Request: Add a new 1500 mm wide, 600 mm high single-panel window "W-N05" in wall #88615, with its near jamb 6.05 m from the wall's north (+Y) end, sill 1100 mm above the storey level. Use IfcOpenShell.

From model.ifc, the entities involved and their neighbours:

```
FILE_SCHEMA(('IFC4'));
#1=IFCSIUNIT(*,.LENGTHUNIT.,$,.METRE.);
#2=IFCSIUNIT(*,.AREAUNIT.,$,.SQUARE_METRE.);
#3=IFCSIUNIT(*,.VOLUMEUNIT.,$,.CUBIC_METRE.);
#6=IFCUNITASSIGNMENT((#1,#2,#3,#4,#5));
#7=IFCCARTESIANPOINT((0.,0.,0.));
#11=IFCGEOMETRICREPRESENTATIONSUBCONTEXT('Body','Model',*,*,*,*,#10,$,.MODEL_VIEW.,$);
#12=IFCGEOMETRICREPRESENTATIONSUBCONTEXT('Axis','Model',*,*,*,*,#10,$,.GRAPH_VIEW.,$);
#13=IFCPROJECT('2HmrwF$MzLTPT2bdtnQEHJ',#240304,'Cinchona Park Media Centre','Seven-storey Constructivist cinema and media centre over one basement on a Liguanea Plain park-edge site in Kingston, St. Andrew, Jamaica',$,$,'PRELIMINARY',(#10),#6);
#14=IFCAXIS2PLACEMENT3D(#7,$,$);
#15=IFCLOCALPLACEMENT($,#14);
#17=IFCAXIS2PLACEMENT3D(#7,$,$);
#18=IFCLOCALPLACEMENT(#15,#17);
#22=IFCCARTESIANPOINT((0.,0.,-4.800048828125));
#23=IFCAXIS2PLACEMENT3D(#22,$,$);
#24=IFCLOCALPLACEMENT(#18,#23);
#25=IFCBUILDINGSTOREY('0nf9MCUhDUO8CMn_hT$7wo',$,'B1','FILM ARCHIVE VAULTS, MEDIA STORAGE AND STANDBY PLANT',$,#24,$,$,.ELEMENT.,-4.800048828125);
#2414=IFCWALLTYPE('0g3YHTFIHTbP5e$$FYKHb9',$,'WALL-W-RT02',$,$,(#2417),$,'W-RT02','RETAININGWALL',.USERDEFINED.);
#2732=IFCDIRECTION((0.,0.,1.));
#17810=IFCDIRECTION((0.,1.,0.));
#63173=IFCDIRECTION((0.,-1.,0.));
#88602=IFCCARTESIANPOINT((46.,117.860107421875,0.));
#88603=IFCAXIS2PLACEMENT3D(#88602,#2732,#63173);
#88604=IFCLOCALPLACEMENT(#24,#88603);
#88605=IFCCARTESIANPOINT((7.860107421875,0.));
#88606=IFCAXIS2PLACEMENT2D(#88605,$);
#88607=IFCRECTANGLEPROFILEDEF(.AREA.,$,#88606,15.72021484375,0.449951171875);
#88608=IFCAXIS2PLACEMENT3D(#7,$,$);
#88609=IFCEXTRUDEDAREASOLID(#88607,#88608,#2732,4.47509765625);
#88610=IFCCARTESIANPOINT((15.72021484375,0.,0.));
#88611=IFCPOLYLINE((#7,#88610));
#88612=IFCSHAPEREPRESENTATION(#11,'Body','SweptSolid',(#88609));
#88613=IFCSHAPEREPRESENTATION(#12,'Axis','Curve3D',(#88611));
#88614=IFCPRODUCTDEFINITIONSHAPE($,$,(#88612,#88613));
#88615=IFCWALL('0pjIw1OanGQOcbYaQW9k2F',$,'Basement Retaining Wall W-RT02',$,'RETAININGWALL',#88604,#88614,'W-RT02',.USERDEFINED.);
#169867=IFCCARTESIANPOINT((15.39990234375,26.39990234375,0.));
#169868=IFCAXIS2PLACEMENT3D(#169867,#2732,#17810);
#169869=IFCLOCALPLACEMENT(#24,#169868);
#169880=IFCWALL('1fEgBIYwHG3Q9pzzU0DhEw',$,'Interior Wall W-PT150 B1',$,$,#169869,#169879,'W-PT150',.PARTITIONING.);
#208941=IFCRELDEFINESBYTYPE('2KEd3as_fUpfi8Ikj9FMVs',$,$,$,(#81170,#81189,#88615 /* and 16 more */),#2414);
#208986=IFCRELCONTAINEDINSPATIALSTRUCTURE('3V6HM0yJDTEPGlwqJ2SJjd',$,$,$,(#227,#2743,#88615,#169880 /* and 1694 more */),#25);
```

```python
import numpy as np
import ifcopenshell
import ifcopenshell.api.feature
import ifcopenshell.api.geometry
import ifcopenshell.api.root
import ifcopenshell.api.spatial
import ifcopenshell.geom
import ifcopenshell.util.element
import ifcopenshell.util.placement
import ifcopenshell.util.representation
import ifcopenshell.util.shape
import ifcopenshell.util.unit

model = ifcopenshell.open("model.ifc")
unit_scale = ifcopenshell.util.unit.calculate_unit_scale(model)
settings = ifcopenshell.geom.settings()


def volume(element):
    """Net volume in cubic metres, openings subtracted."""
    shape = ifcopenshell.geom.create_shape(settings, element)
    return ifcopenshell.util.shape.get_volume(shape.geometry)


wall = model.by_id(88615)
storey = ifcopenshell.util.element.get_container(wall, ifc_class="IfcBuildingStorey")
context = ifcopenshell.util.representation.get_context(model, "Model", "Body", "MODEL_VIEW")
before = volume(wall)

width, height, from_end, sill = 1.5, 0.6, 6.05, 1.1  # metres

# The wall runs along its own X axis, and the end named is its -X end.
wall_shape = ifcopenshell.geom.create_shape(settings, wall)
x, y, z = ifcopenshell.util.shape.get_vertices(wall_shape.geometry).T
start = x.min() + from_end
face, thickness = float(y.min()), float(y.max() - y.min())
wall_matrix = ifcopenshell.util.placement.get_local_placement(wall.ObjectPlacement)
level = ifcopenshell.util.placement.get_local_placement(storey.ObjectPlacement)[2, 3]


def in_wall(x, y):
    """Placement at x, y metres in the wall's axes, at sill height."""
    matrix = wall_matrix.copy()
    matrix[:, 3] = wall_matrix @ np.array([x / unit_scale, y / unit_scale, 0.0, 1.0])
    matrix[2, 3] = level + sill / unit_scale
    return matrix


# Opening: a box that overshoots both wall faces by 50 mm.
opening = ifcopenshell.api.root.create_entity(model, ifc_class="IfcOpeningElement", predefined_type="OPENING")
box = ifcopenshell.api.geometry.add_wall_representation(
    model, context=context, length=width, height=height, thickness=thickness + 0.1
)
ifcopenshell.api.geometry.assign_representation(model, product=opening, representation=box)
ifcopenshell.api.geometry.edit_object_placement(model, product=opening, matrix=in_wall(start, face - 0.05), is_si=False)
ifcopenshell.api.feature.add_feature(model, feature=opening, element=wall)

window = ifcopenshell.api.root.create_entity(model, ifc_class="IfcWindow", name="W-N05", predefined_type="WINDOW")
window.OverallWidth, window.OverallHeight = width / unit_scale, height / unit_scale
window.PartitioningType = "SINGLE_PANEL"
body = ifcopenshell.api.geometry.add_window_representation(
    model,
    context=context,
    overall_width=window.OverallWidth,
    overall_height=window.OverallHeight,
    partition_type="SINGLE_PANEL",
)
ifcopenshell.api.geometry.assign_representation(model, product=window, representation=body)
ifcopenshell.api.spatial.assign_container(model, products=[window], relating_structure=storey)
ifcopenshell.api.feature.add_filling(model, opening=opening, element=window)

# Centre the window in the wall's thickness.
ifcopenshell.api.geometry.edit_object_placement(model, product=window, matrix=in_wall(start, face), is_si=False)
window_shape = ifcopenshell.geom.create_shape(settings, window)
depth = ifcopenshell.util.shape.get_vertices(window_shape.geometry)[:, 1]
offset = face + thickness / 2 - (depth.min() + depth.max()) / 2
ifcopenshell.api.geometry.edit_object_placement(model, product=window, matrix=in_wall(start, offset), is_si=False)

after = volume(wall)

print(f"wall volume {before:.3f} -> {after:.3f} m3")

model.write("model_updated.ifc")
```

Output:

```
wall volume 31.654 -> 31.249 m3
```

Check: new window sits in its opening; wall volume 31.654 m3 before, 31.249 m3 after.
